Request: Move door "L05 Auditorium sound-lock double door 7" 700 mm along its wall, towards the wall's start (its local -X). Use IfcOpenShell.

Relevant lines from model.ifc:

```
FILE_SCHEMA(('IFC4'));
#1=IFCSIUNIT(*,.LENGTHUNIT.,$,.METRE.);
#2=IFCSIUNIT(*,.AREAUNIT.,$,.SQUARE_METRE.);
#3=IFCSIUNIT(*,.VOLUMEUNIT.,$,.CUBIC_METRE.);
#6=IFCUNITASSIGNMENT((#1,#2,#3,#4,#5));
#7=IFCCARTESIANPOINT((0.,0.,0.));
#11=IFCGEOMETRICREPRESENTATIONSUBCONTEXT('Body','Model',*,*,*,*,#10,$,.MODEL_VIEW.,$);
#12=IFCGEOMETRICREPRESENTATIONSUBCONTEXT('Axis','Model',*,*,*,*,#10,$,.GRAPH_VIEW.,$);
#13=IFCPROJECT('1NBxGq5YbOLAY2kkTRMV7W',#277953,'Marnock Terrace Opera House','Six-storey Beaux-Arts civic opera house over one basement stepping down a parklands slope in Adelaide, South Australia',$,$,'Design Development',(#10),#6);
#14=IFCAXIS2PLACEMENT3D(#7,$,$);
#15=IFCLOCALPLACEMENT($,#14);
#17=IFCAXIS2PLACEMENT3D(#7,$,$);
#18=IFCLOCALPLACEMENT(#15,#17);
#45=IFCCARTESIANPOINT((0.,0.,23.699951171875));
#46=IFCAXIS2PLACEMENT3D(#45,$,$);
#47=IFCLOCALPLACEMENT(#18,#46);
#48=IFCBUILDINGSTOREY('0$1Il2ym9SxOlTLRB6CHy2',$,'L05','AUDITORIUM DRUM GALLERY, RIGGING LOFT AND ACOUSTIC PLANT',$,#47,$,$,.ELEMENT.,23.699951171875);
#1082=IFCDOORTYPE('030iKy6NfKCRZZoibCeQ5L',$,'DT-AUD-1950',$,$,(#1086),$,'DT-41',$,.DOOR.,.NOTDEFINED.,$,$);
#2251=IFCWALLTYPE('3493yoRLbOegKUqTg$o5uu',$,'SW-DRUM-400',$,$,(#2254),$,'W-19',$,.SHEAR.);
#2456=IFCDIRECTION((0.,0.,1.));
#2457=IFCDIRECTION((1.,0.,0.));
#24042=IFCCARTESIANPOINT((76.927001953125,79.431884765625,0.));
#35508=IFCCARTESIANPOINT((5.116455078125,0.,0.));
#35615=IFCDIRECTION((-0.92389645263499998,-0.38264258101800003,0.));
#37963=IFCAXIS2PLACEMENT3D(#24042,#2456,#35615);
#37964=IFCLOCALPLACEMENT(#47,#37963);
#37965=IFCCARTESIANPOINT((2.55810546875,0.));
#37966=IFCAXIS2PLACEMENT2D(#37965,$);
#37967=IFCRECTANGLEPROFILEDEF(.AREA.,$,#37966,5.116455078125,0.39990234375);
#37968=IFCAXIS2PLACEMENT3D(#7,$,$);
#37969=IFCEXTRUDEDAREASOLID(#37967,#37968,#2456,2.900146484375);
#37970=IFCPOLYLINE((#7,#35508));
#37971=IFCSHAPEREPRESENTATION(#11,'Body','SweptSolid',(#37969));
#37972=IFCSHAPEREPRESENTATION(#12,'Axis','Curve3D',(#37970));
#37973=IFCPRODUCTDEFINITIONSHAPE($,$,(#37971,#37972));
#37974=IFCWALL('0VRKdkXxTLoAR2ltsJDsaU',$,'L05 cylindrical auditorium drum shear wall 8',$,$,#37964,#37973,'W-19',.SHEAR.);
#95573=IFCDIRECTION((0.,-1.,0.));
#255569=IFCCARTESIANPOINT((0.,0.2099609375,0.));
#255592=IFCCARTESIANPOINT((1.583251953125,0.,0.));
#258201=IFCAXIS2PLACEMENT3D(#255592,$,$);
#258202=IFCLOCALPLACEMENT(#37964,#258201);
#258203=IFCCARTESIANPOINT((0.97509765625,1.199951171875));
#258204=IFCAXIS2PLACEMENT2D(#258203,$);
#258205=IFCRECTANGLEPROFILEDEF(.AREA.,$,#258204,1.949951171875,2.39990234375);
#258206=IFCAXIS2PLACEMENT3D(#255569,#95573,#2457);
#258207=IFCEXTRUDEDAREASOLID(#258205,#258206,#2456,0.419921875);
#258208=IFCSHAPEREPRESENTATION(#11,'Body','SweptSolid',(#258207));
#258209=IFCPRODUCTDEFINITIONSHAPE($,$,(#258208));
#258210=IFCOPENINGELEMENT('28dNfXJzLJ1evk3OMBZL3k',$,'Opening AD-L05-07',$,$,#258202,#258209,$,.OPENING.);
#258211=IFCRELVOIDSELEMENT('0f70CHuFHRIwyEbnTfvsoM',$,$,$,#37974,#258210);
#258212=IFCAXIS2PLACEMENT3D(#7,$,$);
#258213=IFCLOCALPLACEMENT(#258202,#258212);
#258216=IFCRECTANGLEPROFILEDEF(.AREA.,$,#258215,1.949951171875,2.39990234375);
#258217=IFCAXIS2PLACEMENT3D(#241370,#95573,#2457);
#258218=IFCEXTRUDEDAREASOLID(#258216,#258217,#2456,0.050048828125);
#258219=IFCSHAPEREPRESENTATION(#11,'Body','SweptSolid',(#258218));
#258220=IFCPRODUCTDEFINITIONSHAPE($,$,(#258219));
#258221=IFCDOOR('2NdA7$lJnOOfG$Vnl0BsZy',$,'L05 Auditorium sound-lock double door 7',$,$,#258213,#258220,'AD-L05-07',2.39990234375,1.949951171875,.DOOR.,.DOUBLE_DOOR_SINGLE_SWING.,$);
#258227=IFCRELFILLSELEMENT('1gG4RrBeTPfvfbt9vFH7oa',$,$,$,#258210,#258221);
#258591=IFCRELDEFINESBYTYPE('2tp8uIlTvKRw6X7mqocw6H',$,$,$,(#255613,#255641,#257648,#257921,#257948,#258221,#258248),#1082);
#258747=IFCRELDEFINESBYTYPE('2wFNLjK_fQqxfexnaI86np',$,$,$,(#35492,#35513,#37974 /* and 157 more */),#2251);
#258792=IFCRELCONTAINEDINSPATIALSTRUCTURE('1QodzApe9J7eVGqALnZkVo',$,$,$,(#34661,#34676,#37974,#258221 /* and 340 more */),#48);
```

```python
import ifcopenshell
import ifcopenshell.api.geometry
import ifcopenshell.util.placement

model = ifcopenshell.open("model.ifc")

door = model.by_guid("2NdA7$lJnOOfG$Vnl0BsZy")
opening = door.FillsVoids[0].RelatingOpeningElement
wall = opening.VoidsElements[0].RelatingBuildingElement

wall_matrix = ifcopenshell.util.placement.get_local_placement(wall.ObjectPlacement)
shift = wall_matrix[:3, 0] * -0.7
before = ifcopenshell.util.placement.get_local_placement(door.ObjectPlacement)[:3, 3].copy()

# The door is placed relative to its opening, so it follows when the opening moves.
matrix = ifcopenshell.util.placement.get_local_placement(opening.ObjectPlacement)
matrix[:3, 3] += shift
ifcopenshell.api.geometry.edit_object_placement(
    model, product=opening, matrix=matrix, is_si=False, should_transform_children=True
)

after = ifcopenshell.util.placement.get_local_placement(door.ObjectPlacement)[:3, 3]
print("door moved by", (after - before).round(3) + 0.0)

model.write("model_edited.ifc")
```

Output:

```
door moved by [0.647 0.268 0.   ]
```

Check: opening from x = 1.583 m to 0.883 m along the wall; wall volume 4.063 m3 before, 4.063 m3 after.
